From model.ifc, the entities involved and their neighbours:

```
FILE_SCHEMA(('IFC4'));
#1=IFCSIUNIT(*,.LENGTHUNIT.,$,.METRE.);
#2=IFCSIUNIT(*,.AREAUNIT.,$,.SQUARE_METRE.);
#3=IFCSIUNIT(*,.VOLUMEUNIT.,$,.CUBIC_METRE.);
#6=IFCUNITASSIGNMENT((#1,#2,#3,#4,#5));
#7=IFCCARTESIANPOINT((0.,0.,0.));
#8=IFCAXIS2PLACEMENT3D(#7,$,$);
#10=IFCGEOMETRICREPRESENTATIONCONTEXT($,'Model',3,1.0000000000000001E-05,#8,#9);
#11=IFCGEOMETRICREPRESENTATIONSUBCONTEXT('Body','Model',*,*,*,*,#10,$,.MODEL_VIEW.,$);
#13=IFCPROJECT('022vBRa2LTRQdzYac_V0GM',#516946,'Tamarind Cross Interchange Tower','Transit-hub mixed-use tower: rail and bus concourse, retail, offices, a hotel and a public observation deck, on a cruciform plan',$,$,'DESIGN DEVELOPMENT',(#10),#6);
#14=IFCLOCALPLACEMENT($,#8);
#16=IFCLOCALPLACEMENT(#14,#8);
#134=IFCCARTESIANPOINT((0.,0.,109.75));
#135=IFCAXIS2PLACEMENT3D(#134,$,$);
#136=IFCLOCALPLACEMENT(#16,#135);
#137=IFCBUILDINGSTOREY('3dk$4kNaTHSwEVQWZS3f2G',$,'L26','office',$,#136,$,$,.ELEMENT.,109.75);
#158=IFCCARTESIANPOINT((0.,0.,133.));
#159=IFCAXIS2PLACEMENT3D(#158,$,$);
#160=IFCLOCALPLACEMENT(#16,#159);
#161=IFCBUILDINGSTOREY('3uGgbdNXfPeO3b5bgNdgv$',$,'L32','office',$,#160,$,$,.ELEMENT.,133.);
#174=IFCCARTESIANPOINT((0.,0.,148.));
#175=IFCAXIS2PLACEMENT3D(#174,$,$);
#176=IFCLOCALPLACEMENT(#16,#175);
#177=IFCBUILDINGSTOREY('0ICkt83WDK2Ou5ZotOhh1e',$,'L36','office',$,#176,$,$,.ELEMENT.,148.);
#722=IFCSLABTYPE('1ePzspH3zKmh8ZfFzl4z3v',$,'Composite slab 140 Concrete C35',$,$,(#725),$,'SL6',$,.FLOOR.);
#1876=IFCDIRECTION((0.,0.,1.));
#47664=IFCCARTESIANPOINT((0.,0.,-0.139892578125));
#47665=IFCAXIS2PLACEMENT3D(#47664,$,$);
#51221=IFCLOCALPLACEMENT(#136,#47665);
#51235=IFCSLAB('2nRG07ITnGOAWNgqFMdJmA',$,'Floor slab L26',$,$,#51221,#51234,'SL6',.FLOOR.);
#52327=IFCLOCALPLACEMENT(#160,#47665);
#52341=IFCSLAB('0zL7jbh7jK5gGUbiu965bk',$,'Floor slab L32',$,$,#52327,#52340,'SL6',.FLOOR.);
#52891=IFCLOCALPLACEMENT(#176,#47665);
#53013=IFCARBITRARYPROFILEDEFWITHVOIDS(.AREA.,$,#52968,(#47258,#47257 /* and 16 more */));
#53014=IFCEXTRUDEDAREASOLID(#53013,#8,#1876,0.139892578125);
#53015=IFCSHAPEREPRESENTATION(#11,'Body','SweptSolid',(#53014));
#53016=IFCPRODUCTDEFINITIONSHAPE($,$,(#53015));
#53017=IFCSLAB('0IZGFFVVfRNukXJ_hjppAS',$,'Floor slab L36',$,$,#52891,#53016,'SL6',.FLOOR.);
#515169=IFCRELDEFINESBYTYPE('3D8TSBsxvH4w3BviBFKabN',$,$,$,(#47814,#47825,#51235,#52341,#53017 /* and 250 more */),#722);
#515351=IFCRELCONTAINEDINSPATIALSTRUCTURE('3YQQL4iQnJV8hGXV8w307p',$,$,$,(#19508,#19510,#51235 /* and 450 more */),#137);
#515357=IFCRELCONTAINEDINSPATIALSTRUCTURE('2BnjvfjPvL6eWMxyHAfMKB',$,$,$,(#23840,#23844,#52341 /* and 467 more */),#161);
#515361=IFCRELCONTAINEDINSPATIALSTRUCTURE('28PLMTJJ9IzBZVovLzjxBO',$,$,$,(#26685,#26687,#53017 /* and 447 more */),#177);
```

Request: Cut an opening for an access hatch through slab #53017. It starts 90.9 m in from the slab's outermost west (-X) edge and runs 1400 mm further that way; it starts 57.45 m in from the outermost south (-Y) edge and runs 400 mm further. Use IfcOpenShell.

```python
import numpy as np
import ifcopenshell
import ifcopenshell.api.feature
import ifcopenshell.api.geometry
import ifcopenshell.api.root
import ifcopenshell.geom
import ifcopenshell.util.placement
import ifcopenshell.util.representation
import ifcopenshell.util.shape
import ifcopenshell.util.unit

model = ifcopenshell.open("model.ifc")
unit_scale = ifcopenshell.util.unit.calculate_unit_scale(model)
settings = ifcopenshell.geom.settings()


def volume(element):
    """Net volume in cubic metres, openings subtracted."""
    shape = ifcopenshell.geom.create_shape(settings, element)
    return ifcopenshell.util.shape.get_volume(shape.geometry)


slab = model.by_guid("0IZGFFVVfRNukXJ_hjppAS")
before = volume(slab)

# Extent in the slab's own axes, in metres. The edges named are its -X and -Y sides.
slab_shape = ifcopenshell.geom.create_shape(settings, slab)
vertices = ifcopenshell.util.shape.get_vertices(slab_shape.geometry)
x_min, y_min, bottom = vertices.min(axis=0)
top = vertices[:, 2].max()

opening = ifcopenshell.api.root.create_entity(model, ifc_class="IfcOpeningElement", name="Access hatch opening", predefined_type="OPENING")
context = ifcopenshell.util.representation.get_context(model, "Model", "Body", "MODEL_VIEW")
width, depth = 1.4, 0.4
outline = [(0.0, 0.0), (width, 0.0), (width, depth), (0.0, depth), (0.0, 0.0)]
# Overshoot both faces by 50 mm so the cut is clean.
shape = ifcopenshell.api.geometry.add_slab_representation(
    model, context=context, depth=top - bottom + 0.1, polyline=outline
)
ifcopenshell.api.geometry.assign_representation(model, product=opening, representation=shape)

matrix = ifcopenshell.util.placement.get_local_placement(slab.ObjectPlacement)
matrix[:, 3] = matrix @ np.append(np.array([x_min + 90.9, y_min + 57.45, bottom - 0.05]) / unit_scale, 1.0)
ifcopenshell.api.geometry.edit_object_placement(model, product=opening, matrix=matrix, is_si=False)
ifcopenshell.api.feature.add_feature(model, feature=opening, element=slab)

after = volume(slab)

print(f"slab volume {before:.3f} -> {after:.3f} m3")

model.write("model_updated.ifc")
```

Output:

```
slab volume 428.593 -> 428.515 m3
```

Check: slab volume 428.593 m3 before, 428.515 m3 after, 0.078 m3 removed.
